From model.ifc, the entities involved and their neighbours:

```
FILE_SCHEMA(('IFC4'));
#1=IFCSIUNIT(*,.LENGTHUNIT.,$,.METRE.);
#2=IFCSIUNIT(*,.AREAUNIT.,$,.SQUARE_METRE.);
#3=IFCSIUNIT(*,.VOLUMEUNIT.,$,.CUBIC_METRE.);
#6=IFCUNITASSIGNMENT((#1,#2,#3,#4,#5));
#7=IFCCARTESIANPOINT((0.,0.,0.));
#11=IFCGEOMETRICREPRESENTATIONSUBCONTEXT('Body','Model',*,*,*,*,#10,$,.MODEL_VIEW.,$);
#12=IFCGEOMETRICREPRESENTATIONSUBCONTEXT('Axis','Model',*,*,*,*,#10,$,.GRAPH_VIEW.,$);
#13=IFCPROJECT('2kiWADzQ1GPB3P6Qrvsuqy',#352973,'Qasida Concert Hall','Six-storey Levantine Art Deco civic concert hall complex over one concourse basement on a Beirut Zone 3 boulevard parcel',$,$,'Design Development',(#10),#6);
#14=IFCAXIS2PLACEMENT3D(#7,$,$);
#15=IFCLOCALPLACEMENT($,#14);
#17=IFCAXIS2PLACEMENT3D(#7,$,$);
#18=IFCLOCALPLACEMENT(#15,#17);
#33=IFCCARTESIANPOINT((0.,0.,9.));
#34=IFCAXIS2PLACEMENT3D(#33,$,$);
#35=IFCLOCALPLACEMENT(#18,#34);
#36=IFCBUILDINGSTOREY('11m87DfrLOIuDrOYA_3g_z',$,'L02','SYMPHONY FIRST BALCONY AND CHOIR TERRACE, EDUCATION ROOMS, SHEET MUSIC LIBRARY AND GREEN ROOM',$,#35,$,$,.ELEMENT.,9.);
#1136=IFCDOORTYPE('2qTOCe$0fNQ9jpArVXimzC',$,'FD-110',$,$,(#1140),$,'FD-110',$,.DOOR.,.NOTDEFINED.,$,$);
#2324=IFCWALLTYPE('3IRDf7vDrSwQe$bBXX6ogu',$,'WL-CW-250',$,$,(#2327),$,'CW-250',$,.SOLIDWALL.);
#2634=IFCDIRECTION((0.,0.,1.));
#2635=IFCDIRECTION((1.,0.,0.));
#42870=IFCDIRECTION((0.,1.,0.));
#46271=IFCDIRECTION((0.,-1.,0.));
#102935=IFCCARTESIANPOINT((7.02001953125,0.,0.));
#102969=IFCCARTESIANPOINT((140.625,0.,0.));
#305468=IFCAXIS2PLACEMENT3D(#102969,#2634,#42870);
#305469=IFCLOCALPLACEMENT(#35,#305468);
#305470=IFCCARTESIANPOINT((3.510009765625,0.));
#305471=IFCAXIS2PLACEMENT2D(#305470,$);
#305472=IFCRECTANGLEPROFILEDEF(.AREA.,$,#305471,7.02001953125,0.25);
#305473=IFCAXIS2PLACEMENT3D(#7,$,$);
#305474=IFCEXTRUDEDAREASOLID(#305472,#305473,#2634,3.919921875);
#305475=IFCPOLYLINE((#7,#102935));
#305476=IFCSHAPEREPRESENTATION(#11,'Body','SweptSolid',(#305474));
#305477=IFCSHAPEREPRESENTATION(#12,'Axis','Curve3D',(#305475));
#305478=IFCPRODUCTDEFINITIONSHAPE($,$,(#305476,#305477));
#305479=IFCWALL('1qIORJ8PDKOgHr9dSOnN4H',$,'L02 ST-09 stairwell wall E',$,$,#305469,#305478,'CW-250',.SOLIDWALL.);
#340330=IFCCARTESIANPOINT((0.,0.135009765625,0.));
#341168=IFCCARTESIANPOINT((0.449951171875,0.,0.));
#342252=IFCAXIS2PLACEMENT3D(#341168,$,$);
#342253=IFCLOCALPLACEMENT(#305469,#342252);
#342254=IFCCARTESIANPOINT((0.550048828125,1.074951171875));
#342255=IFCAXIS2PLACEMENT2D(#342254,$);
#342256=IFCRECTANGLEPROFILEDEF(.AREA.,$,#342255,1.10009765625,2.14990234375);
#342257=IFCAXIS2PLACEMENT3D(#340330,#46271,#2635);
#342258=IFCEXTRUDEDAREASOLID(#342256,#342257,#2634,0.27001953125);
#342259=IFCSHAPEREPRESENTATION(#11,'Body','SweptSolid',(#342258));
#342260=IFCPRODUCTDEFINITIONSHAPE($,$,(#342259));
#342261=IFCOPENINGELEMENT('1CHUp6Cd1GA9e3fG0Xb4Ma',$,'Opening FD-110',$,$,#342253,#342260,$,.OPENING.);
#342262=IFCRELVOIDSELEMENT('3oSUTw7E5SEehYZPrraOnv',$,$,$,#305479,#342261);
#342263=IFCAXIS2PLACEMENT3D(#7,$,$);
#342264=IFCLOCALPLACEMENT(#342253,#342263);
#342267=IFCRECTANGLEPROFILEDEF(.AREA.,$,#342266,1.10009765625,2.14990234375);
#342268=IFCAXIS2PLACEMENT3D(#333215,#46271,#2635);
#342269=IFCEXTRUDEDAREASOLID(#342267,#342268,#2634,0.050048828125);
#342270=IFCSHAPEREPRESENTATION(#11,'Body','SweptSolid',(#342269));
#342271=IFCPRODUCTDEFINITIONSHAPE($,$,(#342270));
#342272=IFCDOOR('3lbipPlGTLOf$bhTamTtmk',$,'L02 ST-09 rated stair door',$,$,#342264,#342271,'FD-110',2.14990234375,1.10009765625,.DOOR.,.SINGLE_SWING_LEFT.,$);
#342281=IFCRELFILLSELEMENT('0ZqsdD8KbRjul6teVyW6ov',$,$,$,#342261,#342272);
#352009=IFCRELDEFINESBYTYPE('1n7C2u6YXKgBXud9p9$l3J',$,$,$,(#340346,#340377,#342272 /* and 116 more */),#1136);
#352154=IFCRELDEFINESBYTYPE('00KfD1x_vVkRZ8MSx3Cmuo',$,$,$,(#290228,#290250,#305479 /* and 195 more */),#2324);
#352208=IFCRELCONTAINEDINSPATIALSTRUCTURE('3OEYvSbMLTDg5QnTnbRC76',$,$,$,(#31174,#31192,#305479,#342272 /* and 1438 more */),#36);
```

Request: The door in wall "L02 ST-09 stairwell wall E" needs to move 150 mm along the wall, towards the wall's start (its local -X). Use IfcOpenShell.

```python
import ifcopenshell
import ifcopenshell.api.geometry
import ifcopenshell.util.placement

model = ifcopenshell.open("model.ifc")

door = model.by_guid("3lbipPlGTLOf$bhTamTtmk")
opening = door.FillsVoids[0].RelatingOpeningElement
wall = opening.VoidsElements[0].RelatingBuildingElement

wall_matrix = ifcopenshell.util.placement.get_local_placement(wall.ObjectPlacement)
shift = wall_matrix[:3, 0] * -0.15
before = ifcopenshell.util.placement.get_local_placement(door.ObjectPlacement)[:3, 3].copy()

# The door is placed relative to its opening, so it follows when the opening moves.
matrix = ifcopenshell.util.placement.get_local_placement(opening.ObjectPlacement)
matrix[:3, 3] += shift
ifcopenshell.api.geometry.edit_object_placement(
    model, product=opening, matrix=matrix, is_si=False, should_transform_children=True
)

after = ifcopenshell.util.placement.get_local_placement(door.ObjectPlacement)[:3, 3]
print("door moved by", (after - before).round(3) + 0.0)

model.write("model-out.ifc")
```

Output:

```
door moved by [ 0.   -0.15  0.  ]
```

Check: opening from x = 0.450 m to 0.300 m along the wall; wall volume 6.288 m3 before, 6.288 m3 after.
